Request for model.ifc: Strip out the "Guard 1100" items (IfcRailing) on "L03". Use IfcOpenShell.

First a look at what the model holds.

```python
import ifcopenshell
import ifcopenshell.util.element

model = ifcopenshell.open("model.ifc")
print(model.schema)
storey = next(s for s in model.by_type("IfcBuildingStorey") if s.Name == "L03")
railings = [e for e in ifcopenshell.util.element.get_decomposition(storey) if e.is_a("IfcRailing")]
seen = {}
for e in railings:
    element_type = ifcopenshell.util.element.get_type(e)
    name = element_type.Name if element_type not in (None, e) else None
    seen[name] = seen.get(name, 0) + 1
for name, count in sorted(seen.items(), key=str):
    print(count, "x", name)
```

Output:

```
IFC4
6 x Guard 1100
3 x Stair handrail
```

```python
import ifcopenshell
import ifcopenshell.api.root
import ifcopenshell.util.element

model = ifcopenshell.open("model.ifc")

storey = next(s for s in model.by_type("IfcBuildingStorey") if s.Name == "L03")
railings = [e for e in ifcopenshell.util.element.get_decomposition(storey) if e.is_a("IfcRailing")]
targets = [e for e in railings if (t := ifcopenshell.util.element.get_type(e)) not in (None, e) and t.Name == "Guard 1100"]

for e in targets:
    ifcopenshell.api.root.remove_product(model, product=e)
print(len(targets), "removed")

model.write("model_edited.ifc")
```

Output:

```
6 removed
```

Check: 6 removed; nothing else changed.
